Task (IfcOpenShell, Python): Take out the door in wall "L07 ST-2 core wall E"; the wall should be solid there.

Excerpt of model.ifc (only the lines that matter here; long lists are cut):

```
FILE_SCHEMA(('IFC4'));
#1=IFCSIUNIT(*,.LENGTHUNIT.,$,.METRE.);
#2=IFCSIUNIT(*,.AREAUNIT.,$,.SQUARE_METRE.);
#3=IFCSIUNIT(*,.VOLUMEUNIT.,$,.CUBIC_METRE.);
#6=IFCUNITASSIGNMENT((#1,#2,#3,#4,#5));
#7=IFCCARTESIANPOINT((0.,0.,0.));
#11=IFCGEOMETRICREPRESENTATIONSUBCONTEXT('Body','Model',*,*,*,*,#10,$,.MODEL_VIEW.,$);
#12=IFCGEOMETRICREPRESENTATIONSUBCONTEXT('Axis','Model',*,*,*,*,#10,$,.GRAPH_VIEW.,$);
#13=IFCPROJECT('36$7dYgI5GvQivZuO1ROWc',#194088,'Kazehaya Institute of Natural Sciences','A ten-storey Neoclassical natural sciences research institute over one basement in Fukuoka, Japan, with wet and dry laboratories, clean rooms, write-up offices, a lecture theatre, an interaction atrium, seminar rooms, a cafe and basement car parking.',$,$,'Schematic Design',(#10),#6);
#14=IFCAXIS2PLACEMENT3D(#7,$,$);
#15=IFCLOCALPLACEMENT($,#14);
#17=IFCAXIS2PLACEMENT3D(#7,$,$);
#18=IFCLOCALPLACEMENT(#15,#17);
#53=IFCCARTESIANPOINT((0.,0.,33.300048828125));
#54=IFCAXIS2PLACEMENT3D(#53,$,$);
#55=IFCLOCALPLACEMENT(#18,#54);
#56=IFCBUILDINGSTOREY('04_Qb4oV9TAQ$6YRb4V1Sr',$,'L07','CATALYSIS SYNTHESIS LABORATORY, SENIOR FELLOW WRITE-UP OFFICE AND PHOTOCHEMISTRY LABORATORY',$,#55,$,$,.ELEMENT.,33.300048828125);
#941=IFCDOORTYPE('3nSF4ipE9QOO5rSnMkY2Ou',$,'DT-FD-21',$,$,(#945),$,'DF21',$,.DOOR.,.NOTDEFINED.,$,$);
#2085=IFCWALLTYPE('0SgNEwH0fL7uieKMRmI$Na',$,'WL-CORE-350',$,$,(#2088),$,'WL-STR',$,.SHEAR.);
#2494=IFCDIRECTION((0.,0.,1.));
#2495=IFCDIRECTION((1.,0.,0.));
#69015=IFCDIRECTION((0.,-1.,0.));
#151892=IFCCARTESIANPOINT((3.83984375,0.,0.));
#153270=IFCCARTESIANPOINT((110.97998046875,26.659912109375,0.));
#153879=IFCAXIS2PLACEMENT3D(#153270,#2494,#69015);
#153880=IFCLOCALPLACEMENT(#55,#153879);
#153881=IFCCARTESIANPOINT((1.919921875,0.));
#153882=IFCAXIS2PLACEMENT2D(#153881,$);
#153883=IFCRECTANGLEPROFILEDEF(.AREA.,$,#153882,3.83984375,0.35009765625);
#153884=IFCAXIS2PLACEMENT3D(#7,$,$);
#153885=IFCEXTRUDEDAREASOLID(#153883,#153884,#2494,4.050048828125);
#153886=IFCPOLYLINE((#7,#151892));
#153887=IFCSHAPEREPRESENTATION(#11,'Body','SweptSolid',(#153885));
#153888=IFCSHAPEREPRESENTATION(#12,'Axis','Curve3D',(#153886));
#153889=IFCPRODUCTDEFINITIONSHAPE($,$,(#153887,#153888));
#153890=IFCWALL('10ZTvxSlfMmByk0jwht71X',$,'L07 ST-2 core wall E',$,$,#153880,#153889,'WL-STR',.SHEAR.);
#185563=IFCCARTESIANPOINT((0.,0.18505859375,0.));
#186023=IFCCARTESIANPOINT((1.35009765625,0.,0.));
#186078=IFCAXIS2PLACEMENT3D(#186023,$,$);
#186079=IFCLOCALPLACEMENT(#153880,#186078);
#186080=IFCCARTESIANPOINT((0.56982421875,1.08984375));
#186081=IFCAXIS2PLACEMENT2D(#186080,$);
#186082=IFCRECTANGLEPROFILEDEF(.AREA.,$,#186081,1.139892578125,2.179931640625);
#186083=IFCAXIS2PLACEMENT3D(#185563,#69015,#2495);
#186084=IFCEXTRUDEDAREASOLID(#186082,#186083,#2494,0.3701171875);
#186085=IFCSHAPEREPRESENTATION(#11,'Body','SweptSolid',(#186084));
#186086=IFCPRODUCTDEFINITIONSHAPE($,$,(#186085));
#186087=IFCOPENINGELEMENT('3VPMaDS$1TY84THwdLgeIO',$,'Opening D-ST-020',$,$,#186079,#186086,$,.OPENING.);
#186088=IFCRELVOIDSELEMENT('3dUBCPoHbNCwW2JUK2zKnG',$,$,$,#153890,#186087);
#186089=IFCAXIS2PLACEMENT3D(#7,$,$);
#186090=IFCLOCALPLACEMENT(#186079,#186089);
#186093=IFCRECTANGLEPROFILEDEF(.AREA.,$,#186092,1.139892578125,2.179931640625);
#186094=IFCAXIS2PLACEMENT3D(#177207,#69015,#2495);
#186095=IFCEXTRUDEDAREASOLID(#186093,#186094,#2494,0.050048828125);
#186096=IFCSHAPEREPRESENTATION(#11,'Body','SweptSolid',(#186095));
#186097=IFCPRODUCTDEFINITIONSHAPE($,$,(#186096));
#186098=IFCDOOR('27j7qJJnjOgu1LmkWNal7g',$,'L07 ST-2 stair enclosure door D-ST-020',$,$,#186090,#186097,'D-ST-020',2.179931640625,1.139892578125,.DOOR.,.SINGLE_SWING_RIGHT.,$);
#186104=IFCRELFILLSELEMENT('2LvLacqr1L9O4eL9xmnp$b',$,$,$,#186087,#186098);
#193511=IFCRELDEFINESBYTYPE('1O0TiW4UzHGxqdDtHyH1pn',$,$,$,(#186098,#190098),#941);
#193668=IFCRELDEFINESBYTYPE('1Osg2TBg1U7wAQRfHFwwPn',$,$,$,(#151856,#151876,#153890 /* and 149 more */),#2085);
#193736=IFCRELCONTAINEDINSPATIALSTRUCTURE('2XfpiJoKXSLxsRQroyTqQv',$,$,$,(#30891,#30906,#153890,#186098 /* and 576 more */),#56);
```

```python
import ifcopenshell
import ifcopenshell.api.feature
import ifcopenshell.api.root
import ifcopenshell.geom
import ifcopenshell.util.shape

model = ifcopenshell.open("model.ifc")
settings = ifcopenshell.geom.settings()


def volume(element):
    """Net volume in cubic metres, openings subtracted."""
    shape = ifcopenshell.geom.create_shape(settings, element)
    return ifcopenshell.util.shape.get_volume(shape.geometry)


door = model.by_guid("27j7qJJnjOgu1LmkWNal7g")
opening = door.FillsVoids[0].RelatingOpeningElement
wall = opening.VoidsElements[0].RelatingBuildingElement
before = volume(wall)

ifcopenshell.api.root.remove_product(model, product=door)
ifcopenshell.api.feature.remove_feature(model, feature=opening)

after = volume(wall)

print(f"wall volume {before:.3f} -> {after:.3f} m3")

model.write("model_edited.ifc")
```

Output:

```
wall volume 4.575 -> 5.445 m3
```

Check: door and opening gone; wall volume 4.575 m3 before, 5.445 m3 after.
